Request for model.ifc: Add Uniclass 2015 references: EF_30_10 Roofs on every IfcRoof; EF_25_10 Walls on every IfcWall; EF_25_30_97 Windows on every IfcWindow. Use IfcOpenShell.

First a look at what the model holds.

```python
import ifcopenshell

model = ifcopenshell.open("model.ifc")
print(model.schema)
print("classifications:", [c.Name for c in model.by_type("IfcClassification")])
for ifc_class in ("IfcDoor", "IfcRoof", "IfcStair", "IfcWall", "IfcWindow"):
    print(ifc_class, len(model.by_type(ifc_class)))
```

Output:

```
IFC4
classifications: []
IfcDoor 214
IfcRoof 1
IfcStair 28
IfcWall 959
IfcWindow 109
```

```python
import ifcopenshell
import ifcopenshell.api.classification

model = ifcopenshell.open("model.ifc")

system = ifcopenshell.api.classification.add_classification(model, classification="Uniclass 2015")

codes = {
    "IfcRoof": ("EF_30_10", "Roofs"),
    "IfcWall": ("EF_25_10", "Walls"),
    "IfcWindow": ("EF_25_30_97", "Windows"),
}
for ifc_class, (code, name) in codes.items():
    products = model.by_type(ifc_class)
    ifcopenshell.api.classification.add_reference(
        model, products=products, classification=system, identification=code, name=name
    )
    print(code, len(products))

model.write("model_v2.ifc")
```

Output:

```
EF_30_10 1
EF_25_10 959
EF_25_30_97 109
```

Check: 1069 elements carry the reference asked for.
